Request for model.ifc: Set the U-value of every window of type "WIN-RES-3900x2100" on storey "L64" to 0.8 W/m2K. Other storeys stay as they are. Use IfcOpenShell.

First a look at what the model holds.

```python
import ifcopenshell
import ifcopenshell.util.element

model = ifcopenshell.open("model.ifc")
print(model.schema)
storey = next(s for s in model.by_type("IfcBuildingStorey") if s.Name == "L64")
windows = [e for e in ifcopenshell.util.element.get_decomposition(storey) if e.is_a("IfcWindow")]
seen = {}
for e in windows:
    element_type = ifcopenshell.util.element.get_type(e)
    key = (element_type.Name if element_type != e and element_type else None, ifcopenshell.util.element.get_pset(e, "Pset_WindowCommon", "ThermalTransmittance"))
    seen[key] = seen.get(key, 0) + 1
for (name, value), count in sorted(seen.items(), key=str):
    print(count, "x", name, "|", value)
```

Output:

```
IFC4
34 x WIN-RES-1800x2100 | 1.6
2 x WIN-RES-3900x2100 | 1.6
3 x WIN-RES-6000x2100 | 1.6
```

```python
import ifcopenshell
import ifcopenshell.api.pset
import ifcopenshell.util.element

model = ifcopenshell.open("model.ifc")

storey = next(s for s in model.by_type("IfcBuildingStorey") if s.Name == "L64")
windows = [e for e in ifcopenshell.util.element.get_decomposition(storey) if e.is_a("IfcWindow")]

count = 0
for e in windows:
    element_type = ifcopenshell.util.element.get_type(e)
    if element_type in (None, e) or element_type.Name != "WIN-RES-3900x2100":
        continue
    found = ifcopenshell.util.element.get_pset(e, "Pset_WindowCommon", should_inherit=False)
    if found:
        pset = model.by_id(found["id"])
        if len(ifcopenshell.util.element.get_elements_by_pset(pset)) > 1:
            pset = ifcopenshell.api.pset.unshare_pset(model, products=[e], pset=pset)[0]
    else:
        pset = ifcopenshell.api.pset.add_pset(model, product=e, name="Pset_WindowCommon")
    ifcopenshell.api.pset.edit_pset(model, pset=pset, properties={"ThermalTransmittance": 0.8})
    count += 1

print(count, "windows updated")

model.write("model_edited.ifc")
```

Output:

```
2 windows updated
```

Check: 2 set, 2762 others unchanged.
